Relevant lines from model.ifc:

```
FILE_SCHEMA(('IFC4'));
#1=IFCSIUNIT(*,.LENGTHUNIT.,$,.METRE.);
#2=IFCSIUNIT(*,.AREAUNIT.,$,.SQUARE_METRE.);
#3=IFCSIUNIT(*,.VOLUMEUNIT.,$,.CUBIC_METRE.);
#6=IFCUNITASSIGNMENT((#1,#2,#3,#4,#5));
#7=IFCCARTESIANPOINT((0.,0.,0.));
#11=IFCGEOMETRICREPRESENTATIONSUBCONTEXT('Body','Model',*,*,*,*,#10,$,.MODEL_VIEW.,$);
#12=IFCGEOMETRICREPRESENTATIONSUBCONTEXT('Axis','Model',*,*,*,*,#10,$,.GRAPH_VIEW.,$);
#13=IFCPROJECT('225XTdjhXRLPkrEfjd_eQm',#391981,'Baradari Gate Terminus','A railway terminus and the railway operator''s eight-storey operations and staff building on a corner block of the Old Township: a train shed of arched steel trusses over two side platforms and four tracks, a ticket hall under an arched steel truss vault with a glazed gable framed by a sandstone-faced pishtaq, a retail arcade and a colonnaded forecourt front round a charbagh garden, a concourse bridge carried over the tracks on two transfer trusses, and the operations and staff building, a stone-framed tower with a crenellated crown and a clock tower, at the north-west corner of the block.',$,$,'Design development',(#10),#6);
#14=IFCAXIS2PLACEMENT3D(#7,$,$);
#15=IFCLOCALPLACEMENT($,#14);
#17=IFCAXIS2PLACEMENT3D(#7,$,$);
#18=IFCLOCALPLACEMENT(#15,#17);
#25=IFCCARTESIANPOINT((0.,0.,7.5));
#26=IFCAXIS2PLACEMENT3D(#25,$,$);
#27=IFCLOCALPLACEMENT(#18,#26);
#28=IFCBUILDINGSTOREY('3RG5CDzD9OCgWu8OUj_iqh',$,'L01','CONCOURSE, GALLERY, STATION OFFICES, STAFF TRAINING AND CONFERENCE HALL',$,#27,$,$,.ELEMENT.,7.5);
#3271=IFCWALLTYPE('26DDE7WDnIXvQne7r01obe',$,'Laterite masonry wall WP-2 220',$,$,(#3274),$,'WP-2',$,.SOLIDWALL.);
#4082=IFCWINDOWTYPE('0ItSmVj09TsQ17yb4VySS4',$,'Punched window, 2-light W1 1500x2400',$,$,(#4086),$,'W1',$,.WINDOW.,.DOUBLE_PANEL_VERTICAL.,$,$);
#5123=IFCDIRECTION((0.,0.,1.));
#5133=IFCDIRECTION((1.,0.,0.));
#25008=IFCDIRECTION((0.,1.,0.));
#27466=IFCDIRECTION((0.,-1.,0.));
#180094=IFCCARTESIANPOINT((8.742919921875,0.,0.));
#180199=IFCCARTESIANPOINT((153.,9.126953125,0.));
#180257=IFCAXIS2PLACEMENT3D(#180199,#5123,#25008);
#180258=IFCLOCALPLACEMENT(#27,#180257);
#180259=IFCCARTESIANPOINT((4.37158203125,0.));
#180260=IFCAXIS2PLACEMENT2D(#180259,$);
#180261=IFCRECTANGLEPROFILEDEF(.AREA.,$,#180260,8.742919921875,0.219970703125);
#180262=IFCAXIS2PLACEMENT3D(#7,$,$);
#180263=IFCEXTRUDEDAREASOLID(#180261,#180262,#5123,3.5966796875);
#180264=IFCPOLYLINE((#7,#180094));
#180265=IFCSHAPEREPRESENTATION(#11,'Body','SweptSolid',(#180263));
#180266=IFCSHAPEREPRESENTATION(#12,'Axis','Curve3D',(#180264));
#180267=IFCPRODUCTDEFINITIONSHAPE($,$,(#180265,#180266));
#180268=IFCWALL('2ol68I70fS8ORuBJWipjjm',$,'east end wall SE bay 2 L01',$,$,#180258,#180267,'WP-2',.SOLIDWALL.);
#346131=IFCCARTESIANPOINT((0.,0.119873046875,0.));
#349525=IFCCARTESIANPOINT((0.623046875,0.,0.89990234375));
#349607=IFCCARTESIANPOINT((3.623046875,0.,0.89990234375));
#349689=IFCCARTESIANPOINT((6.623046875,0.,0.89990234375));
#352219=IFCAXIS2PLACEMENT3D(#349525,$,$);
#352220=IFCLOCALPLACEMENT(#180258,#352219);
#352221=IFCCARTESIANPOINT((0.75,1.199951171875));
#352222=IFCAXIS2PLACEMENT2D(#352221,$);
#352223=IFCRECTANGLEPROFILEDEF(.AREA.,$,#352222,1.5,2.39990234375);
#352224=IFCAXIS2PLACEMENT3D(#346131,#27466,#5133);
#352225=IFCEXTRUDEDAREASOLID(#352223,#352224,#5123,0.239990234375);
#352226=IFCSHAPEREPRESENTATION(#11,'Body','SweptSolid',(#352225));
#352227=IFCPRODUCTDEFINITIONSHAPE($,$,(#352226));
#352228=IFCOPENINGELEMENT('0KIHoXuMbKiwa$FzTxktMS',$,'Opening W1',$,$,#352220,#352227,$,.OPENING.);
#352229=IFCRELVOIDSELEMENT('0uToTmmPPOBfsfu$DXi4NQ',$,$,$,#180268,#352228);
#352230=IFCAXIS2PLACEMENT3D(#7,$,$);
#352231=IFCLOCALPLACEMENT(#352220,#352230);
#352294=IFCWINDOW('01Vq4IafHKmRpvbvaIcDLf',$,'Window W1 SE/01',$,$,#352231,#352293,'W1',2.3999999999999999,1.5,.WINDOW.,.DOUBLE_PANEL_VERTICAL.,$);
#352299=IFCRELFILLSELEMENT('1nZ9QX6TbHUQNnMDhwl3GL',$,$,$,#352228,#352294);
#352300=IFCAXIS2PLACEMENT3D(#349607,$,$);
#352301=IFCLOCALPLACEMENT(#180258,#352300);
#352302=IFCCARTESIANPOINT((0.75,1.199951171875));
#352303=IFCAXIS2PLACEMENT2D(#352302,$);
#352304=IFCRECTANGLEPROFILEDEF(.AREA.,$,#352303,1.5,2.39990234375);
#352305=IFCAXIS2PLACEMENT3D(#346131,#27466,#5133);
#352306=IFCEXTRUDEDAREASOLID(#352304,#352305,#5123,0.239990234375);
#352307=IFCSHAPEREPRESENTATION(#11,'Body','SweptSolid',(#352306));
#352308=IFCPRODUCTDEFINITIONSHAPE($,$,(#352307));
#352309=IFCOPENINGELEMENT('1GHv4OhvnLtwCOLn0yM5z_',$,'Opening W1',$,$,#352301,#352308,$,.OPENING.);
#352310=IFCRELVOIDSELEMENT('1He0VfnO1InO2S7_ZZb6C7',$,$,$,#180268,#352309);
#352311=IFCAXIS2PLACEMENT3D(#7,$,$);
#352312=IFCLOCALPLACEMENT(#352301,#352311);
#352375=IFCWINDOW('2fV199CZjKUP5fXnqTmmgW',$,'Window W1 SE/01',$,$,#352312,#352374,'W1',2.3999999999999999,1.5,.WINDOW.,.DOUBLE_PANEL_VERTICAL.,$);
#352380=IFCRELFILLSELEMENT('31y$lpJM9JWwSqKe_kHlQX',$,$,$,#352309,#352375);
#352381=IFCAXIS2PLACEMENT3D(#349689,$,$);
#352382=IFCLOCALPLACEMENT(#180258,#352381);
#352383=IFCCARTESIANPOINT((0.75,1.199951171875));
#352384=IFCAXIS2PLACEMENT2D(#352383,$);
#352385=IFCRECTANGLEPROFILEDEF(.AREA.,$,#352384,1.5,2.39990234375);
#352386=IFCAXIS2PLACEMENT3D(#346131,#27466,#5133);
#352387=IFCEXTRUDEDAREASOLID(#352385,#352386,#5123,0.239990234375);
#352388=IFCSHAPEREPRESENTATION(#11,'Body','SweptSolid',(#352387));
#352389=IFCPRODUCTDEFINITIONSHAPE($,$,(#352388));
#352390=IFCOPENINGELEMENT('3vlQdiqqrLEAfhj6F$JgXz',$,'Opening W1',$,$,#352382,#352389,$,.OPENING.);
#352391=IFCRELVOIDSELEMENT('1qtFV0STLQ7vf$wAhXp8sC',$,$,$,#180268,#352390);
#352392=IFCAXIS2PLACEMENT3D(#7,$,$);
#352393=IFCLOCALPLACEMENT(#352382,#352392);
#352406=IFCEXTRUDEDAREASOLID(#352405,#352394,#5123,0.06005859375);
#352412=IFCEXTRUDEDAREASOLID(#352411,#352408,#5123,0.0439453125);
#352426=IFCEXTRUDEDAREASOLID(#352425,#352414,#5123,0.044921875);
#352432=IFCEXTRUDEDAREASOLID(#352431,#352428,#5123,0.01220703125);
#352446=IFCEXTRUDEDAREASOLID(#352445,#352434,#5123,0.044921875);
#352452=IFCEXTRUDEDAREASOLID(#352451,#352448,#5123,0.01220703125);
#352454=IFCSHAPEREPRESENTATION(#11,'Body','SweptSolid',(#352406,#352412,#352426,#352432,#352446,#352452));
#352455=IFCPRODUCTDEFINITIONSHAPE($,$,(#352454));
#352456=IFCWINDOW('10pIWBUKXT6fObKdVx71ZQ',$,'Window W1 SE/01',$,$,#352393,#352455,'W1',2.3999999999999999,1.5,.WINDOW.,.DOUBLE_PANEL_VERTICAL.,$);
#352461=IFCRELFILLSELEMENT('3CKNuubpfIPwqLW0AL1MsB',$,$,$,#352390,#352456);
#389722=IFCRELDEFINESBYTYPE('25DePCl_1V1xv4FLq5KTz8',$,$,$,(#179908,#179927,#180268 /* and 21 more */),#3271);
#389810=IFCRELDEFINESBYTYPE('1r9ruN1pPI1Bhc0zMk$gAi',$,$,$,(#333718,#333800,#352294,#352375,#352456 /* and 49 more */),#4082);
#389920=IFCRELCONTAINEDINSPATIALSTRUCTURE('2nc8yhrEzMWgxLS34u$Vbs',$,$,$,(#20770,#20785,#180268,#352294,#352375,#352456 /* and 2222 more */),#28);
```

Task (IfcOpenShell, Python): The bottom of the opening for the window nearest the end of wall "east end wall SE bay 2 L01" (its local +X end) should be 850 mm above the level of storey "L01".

```python
import numpy as np
import ifcopenshell
import ifcopenshell.api.geometry
import ifcopenshell.geom
import ifcopenshell.util.element
import ifcopenshell.util.placement
import ifcopenshell.util.shape
import ifcopenshell.util.unit

model = ifcopenshell.open("model.ifc")
unit_scale = ifcopenshell.util.unit.calculate_unit_scale(model)

window = model.by_id(352456)
opening = window.FillsVoids[0].RelatingOpeningElement
storey = ifcopenshell.util.element.get_container(window, ifc_class="IfcBuildingStorey")
level = ifcopenshell.util.placement.get_local_placement(storey.ObjectPlacement)[2, 3]

# The opening's origin need not be at the sill, so measure its lowest point.
shape = ifcopenshell.geom.create_shape(ifcopenshell.geom.settings(), opening)
bottom = ifcopenshell.util.shape.get_shape_bottom_elevation(shape, shape.geometry) / unit_scale
dz = level + 0.85 / unit_scale - bottom

shift = np.array([0.0, 0.0, dz])
# The window is placed relative to its opening, so it follows when the opening moves.
matrix = ifcopenshell.util.placement.get_local_placement(opening.ObjectPlacement)
matrix[:3, 3] += shift
ifcopenshell.api.geometry.edit_object_placement(
    model, product=opening, matrix=matrix, is_si=False, should_transform_children=True
)

print(f"moved by {dz * unit_scale:+.3f} m")

model.write("model-out.ifc")
```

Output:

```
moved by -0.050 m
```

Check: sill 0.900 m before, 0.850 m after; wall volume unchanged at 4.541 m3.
